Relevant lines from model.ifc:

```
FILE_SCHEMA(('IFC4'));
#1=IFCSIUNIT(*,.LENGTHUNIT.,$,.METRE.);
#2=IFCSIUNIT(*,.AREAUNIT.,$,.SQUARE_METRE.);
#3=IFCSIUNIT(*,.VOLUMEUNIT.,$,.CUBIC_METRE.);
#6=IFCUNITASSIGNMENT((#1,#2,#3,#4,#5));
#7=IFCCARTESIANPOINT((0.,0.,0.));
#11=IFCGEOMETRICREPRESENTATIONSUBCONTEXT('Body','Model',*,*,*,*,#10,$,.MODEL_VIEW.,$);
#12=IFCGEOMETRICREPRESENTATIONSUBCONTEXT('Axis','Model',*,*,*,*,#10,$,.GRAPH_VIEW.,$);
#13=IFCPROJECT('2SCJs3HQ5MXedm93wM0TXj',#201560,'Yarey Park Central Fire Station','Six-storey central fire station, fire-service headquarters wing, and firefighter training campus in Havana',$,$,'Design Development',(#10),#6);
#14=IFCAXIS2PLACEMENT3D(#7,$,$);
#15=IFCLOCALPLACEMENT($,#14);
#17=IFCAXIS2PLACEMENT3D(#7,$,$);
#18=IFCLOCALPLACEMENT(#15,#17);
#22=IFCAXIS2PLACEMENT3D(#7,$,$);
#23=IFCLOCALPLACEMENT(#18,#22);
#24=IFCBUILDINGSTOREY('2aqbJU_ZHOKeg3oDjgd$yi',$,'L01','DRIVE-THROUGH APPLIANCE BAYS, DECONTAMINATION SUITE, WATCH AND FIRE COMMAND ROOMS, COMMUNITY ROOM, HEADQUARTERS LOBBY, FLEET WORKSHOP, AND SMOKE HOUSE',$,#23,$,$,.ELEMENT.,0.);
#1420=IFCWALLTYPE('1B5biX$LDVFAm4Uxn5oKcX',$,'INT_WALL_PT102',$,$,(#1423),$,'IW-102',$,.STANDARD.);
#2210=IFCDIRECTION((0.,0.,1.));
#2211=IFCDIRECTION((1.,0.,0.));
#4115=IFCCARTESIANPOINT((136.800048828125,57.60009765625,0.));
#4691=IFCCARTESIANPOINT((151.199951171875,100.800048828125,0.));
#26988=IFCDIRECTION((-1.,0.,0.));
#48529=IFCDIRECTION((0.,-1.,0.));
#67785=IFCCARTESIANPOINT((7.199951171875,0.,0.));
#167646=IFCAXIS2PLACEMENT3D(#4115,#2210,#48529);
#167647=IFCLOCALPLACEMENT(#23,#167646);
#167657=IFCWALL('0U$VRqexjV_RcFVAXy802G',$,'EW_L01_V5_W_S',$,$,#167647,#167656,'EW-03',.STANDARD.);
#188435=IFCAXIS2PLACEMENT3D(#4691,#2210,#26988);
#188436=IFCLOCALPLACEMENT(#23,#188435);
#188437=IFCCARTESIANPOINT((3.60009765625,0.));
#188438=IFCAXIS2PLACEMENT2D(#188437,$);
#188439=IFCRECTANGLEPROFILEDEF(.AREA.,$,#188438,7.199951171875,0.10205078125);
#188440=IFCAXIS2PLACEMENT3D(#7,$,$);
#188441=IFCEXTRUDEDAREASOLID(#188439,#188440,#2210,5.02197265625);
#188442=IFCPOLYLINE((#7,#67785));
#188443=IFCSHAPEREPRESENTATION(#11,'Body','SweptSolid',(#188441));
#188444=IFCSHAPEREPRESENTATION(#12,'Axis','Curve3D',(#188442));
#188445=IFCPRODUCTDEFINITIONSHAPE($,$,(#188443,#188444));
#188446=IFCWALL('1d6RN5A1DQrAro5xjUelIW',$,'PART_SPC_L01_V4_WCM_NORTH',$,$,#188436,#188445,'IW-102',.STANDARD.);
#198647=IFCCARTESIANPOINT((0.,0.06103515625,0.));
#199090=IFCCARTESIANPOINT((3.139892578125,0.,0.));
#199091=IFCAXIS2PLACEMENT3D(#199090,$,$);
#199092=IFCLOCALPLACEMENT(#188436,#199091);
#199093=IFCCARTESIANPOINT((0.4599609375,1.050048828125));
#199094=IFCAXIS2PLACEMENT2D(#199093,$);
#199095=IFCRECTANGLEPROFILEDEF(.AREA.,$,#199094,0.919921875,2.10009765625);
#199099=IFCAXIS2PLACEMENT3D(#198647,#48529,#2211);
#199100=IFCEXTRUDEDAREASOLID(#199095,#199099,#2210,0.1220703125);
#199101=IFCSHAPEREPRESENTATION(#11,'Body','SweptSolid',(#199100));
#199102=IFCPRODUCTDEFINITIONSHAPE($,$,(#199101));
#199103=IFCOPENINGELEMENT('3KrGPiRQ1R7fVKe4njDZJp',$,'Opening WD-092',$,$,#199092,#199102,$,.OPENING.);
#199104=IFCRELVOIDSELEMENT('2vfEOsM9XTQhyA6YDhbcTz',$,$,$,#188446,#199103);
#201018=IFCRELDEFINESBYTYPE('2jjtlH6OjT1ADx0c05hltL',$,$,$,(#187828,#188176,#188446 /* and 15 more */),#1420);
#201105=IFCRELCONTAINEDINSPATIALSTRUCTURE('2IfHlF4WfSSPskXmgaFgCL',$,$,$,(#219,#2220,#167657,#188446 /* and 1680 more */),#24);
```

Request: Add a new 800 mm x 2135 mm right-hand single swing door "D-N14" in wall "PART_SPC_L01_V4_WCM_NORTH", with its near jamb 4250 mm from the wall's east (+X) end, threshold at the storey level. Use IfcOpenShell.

```python
import numpy as np
import ifcopenshell
import ifcopenshell.api.feature
import ifcopenshell.api.geometry
import ifcopenshell.api.root
import ifcopenshell.api.spatial
import ifcopenshell.geom
import ifcopenshell.util.element
import ifcopenshell.util.placement
import ifcopenshell.util.representation
import ifcopenshell.util.shape
import ifcopenshell.util.unit

model = ifcopenshell.open("model.ifc")
unit_scale = ifcopenshell.util.unit.calculate_unit_scale(model)
settings = ifcopenshell.geom.settings()


def volume(element):
    """Net volume in cubic metres, openings subtracted."""
    shape = ifcopenshell.geom.create_shape(settings, element)
    return ifcopenshell.util.shape.get_volume(shape.geometry)


wall = model.by_guid("1d6RN5A1DQrAro5xjUelIW")
storey = ifcopenshell.util.element.get_container(wall, ifc_class="IfcBuildingStorey")
context = ifcopenshell.util.representation.get_context(model, "Model", "Body", "MODEL_VIEW")
before = volume(wall)

width, height, from_end, sill = 0.8, 2.135, 4.25, 0.0  # metres

# The wall runs along its own X axis, and the end named is its -X end.
wall_shape = ifcopenshell.geom.create_shape(settings, wall)
x, y, z = ifcopenshell.util.shape.get_vertices(wall_shape.geometry).T
start = x.min() + from_end
face, thickness = float(y.min()), float(y.max() - y.min())
wall_matrix = ifcopenshell.util.placement.get_local_placement(wall.ObjectPlacement)
level = ifcopenshell.util.placement.get_local_placement(storey.ObjectPlacement)[2, 3]


def in_wall(x, y):
    """Placement at x, y metres in the wall's axes, at sill height."""
    matrix = wall_matrix.copy()
    matrix[:, 3] = wall_matrix @ np.array([x / unit_scale, y / unit_scale, 0.0, 1.0])
    matrix[2, 3] = level + sill / unit_scale
    return matrix


# Opening: a box that overshoots both wall faces by 50 mm.
opening = ifcopenshell.api.root.create_entity(model, ifc_class="IfcOpeningElement", predefined_type="OPENING")
box = ifcopenshell.api.geometry.add_wall_representation(
    model, context=context, length=width, height=height, thickness=thickness + 0.1
)
ifcopenshell.api.geometry.assign_representation(model, product=opening, representation=box)
ifcopenshell.api.geometry.edit_object_placement(model, product=opening, matrix=in_wall(start, face - 0.05), is_si=False)
ifcopenshell.api.feature.add_feature(model, feature=opening, element=wall)

door = ifcopenshell.api.root.create_entity(model, ifc_class="IfcDoor", name="D-N14", predefined_type="DOOR")
door.OverallWidth, door.OverallHeight = width / unit_scale, height / unit_scale
door.OperationType = "SINGLE_SWING_RIGHT"
body = ifcopenshell.api.geometry.add_door_representation(
    model,
    context=context,
    overall_width=door.OverallWidth,
    overall_height=door.OverallHeight,
    operation_type="SINGLE_SWING_RIGHT",
    lining_properties={"LiningDepth": thickness / unit_scale, "ThresholdDepth": thickness / unit_scale},
)
ifcopenshell.api.geometry.assign_representation(model, product=door, representation=body)
ifcopenshell.api.spatial.assign_container(model, products=[door], relating_structure=storey)
ifcopenshell.api.feature.add_filling(model, opening=opening, element=door)

# The lining spans the wall, so the door starts at the wall face.
ifcopenshell.api.geometry.edit_object_placement(model, product=door, matrix=in_wall(start, face), is_si=False)

after = volume(wall)

print(f"wall volume {before:.3f} -> {after:.3f} m3")

model.write("model_updated.ifc")
```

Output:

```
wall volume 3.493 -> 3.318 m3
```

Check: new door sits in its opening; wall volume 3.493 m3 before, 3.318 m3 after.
